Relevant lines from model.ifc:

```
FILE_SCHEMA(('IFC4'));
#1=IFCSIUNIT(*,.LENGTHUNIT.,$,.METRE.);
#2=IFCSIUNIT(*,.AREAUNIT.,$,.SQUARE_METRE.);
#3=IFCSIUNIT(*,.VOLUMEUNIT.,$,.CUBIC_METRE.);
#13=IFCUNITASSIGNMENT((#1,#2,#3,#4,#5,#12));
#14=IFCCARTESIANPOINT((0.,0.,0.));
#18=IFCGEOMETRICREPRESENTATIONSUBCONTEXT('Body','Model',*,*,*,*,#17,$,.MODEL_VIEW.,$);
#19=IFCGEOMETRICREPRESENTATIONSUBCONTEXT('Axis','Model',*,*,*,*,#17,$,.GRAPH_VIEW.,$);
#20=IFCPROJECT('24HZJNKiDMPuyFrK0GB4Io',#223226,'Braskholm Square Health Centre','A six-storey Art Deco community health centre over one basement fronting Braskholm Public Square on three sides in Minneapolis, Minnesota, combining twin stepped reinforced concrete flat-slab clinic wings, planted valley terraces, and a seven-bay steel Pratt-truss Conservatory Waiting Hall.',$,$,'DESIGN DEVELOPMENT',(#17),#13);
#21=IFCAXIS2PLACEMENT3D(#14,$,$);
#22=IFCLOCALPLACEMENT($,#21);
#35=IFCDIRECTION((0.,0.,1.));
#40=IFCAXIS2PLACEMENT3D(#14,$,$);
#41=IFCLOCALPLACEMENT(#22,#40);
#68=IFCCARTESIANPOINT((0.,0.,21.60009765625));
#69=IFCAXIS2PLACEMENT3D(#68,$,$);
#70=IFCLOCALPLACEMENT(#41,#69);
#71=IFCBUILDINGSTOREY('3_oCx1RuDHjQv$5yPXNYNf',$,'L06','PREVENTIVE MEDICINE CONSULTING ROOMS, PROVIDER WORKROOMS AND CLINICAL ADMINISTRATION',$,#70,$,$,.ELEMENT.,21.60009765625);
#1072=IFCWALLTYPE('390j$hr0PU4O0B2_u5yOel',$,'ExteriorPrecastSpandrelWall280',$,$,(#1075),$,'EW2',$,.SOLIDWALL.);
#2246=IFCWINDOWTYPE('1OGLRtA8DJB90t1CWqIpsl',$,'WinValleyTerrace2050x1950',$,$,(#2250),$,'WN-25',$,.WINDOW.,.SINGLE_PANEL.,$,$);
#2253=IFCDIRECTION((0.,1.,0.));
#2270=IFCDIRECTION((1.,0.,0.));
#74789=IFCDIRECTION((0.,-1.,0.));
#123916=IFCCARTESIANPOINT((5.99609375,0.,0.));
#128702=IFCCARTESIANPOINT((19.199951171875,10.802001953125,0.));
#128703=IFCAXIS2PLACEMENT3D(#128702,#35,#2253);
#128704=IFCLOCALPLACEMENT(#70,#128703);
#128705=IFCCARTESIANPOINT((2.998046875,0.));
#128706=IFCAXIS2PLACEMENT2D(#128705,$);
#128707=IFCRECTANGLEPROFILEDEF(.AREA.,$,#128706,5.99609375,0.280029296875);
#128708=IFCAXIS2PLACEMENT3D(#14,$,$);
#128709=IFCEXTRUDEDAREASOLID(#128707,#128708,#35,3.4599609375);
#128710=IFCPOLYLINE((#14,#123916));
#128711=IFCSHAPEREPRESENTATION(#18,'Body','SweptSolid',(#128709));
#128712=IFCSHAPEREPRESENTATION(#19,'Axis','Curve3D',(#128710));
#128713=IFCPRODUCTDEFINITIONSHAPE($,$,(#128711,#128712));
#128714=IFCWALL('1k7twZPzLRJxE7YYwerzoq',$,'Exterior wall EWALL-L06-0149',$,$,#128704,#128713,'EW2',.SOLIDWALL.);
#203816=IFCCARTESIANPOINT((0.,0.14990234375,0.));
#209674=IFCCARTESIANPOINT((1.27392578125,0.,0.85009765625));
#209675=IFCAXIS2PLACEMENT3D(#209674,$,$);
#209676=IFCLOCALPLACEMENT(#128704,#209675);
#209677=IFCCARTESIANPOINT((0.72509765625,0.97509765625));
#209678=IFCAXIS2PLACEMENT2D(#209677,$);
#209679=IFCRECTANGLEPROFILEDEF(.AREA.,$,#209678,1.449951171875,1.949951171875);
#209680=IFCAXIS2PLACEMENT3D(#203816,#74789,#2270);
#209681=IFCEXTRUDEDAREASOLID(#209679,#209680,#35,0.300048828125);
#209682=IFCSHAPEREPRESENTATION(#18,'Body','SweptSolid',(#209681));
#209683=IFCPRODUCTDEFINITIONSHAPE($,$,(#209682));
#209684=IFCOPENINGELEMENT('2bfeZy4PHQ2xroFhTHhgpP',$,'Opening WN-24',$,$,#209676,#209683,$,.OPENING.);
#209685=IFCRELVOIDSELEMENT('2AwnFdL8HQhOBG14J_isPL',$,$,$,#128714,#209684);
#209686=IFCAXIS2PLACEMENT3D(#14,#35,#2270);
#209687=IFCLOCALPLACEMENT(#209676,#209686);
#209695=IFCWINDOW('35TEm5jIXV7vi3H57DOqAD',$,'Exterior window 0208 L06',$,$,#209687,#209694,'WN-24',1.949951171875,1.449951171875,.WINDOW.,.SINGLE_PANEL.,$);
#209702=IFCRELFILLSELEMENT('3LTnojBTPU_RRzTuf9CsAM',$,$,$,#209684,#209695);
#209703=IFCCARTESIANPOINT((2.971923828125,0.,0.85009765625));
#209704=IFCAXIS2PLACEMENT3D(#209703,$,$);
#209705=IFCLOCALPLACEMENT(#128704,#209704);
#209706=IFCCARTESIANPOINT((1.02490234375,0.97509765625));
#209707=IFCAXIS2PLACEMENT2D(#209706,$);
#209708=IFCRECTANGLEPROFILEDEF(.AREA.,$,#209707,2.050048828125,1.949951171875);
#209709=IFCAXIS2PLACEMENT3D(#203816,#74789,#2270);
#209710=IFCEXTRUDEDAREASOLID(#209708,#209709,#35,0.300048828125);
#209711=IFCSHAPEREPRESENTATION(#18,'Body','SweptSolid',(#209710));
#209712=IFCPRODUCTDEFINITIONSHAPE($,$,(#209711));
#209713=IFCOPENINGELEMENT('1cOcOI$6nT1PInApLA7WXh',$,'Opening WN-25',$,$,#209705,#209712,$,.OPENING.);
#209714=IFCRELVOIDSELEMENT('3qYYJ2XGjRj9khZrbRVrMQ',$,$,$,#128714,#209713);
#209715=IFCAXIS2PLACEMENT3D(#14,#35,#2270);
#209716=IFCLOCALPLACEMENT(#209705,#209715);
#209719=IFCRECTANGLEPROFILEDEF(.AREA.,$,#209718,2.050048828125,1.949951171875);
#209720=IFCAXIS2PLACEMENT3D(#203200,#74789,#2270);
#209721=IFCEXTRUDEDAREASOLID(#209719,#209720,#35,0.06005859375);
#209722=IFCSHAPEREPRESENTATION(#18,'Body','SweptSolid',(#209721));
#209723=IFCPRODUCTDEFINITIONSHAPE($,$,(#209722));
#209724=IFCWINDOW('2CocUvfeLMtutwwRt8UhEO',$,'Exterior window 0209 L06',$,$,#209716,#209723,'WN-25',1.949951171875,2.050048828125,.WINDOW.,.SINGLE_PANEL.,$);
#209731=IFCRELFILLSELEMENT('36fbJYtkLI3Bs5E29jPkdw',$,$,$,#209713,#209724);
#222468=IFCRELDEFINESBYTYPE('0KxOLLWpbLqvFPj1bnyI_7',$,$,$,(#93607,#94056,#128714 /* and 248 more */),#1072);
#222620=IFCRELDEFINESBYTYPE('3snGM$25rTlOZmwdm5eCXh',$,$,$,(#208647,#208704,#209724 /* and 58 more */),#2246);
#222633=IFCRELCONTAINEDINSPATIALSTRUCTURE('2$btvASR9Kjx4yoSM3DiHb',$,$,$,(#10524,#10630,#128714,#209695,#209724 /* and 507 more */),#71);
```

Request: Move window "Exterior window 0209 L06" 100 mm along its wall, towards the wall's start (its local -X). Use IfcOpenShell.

```python
import ifcopenshell
import ifcopenshell.api.geometry
import ifcopenshell.util.placement

model = ifcopenshell.open("model.ifc")

window = model.by_guid("2CocUvfeLMtutwwRt8UhEO")
opening = window.FillsVoids[0].RelatingOpeningElement
wall = opening.VoidsElements[0].RelatingBuildingElement

wall_matrix = ifcopenshell.util.placement.get_local_placement(wall.ObjectPlacement)
shift = wall_matrix[:3, 0] * -0.1
before = ifcopenshell.util.placement.get_local_placement(window.ObjectPlacement)[:3, 3].copy()

# The window is placed relative to its opening, so it follows when the opening moves.
matrix = ifcopenshell.util.placement.get_local_placement(opening.ObjectPlacement)
matrix[:3, 3] += shift
ifcopenshell.api.geometry.edit_object_placement(
    model, product=opening, matrix=matrix, is_si=False, should_transform_children=True
)

after = ifcopenshell.util.placement.get_local_placement(window.ObjectPlacement)[:3, 3]
print("window moved by", (after - before).round(3) + 0.0)

model.write("model_rev.ifc")
```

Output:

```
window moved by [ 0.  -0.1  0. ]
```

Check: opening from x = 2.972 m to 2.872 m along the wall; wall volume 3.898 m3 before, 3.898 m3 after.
